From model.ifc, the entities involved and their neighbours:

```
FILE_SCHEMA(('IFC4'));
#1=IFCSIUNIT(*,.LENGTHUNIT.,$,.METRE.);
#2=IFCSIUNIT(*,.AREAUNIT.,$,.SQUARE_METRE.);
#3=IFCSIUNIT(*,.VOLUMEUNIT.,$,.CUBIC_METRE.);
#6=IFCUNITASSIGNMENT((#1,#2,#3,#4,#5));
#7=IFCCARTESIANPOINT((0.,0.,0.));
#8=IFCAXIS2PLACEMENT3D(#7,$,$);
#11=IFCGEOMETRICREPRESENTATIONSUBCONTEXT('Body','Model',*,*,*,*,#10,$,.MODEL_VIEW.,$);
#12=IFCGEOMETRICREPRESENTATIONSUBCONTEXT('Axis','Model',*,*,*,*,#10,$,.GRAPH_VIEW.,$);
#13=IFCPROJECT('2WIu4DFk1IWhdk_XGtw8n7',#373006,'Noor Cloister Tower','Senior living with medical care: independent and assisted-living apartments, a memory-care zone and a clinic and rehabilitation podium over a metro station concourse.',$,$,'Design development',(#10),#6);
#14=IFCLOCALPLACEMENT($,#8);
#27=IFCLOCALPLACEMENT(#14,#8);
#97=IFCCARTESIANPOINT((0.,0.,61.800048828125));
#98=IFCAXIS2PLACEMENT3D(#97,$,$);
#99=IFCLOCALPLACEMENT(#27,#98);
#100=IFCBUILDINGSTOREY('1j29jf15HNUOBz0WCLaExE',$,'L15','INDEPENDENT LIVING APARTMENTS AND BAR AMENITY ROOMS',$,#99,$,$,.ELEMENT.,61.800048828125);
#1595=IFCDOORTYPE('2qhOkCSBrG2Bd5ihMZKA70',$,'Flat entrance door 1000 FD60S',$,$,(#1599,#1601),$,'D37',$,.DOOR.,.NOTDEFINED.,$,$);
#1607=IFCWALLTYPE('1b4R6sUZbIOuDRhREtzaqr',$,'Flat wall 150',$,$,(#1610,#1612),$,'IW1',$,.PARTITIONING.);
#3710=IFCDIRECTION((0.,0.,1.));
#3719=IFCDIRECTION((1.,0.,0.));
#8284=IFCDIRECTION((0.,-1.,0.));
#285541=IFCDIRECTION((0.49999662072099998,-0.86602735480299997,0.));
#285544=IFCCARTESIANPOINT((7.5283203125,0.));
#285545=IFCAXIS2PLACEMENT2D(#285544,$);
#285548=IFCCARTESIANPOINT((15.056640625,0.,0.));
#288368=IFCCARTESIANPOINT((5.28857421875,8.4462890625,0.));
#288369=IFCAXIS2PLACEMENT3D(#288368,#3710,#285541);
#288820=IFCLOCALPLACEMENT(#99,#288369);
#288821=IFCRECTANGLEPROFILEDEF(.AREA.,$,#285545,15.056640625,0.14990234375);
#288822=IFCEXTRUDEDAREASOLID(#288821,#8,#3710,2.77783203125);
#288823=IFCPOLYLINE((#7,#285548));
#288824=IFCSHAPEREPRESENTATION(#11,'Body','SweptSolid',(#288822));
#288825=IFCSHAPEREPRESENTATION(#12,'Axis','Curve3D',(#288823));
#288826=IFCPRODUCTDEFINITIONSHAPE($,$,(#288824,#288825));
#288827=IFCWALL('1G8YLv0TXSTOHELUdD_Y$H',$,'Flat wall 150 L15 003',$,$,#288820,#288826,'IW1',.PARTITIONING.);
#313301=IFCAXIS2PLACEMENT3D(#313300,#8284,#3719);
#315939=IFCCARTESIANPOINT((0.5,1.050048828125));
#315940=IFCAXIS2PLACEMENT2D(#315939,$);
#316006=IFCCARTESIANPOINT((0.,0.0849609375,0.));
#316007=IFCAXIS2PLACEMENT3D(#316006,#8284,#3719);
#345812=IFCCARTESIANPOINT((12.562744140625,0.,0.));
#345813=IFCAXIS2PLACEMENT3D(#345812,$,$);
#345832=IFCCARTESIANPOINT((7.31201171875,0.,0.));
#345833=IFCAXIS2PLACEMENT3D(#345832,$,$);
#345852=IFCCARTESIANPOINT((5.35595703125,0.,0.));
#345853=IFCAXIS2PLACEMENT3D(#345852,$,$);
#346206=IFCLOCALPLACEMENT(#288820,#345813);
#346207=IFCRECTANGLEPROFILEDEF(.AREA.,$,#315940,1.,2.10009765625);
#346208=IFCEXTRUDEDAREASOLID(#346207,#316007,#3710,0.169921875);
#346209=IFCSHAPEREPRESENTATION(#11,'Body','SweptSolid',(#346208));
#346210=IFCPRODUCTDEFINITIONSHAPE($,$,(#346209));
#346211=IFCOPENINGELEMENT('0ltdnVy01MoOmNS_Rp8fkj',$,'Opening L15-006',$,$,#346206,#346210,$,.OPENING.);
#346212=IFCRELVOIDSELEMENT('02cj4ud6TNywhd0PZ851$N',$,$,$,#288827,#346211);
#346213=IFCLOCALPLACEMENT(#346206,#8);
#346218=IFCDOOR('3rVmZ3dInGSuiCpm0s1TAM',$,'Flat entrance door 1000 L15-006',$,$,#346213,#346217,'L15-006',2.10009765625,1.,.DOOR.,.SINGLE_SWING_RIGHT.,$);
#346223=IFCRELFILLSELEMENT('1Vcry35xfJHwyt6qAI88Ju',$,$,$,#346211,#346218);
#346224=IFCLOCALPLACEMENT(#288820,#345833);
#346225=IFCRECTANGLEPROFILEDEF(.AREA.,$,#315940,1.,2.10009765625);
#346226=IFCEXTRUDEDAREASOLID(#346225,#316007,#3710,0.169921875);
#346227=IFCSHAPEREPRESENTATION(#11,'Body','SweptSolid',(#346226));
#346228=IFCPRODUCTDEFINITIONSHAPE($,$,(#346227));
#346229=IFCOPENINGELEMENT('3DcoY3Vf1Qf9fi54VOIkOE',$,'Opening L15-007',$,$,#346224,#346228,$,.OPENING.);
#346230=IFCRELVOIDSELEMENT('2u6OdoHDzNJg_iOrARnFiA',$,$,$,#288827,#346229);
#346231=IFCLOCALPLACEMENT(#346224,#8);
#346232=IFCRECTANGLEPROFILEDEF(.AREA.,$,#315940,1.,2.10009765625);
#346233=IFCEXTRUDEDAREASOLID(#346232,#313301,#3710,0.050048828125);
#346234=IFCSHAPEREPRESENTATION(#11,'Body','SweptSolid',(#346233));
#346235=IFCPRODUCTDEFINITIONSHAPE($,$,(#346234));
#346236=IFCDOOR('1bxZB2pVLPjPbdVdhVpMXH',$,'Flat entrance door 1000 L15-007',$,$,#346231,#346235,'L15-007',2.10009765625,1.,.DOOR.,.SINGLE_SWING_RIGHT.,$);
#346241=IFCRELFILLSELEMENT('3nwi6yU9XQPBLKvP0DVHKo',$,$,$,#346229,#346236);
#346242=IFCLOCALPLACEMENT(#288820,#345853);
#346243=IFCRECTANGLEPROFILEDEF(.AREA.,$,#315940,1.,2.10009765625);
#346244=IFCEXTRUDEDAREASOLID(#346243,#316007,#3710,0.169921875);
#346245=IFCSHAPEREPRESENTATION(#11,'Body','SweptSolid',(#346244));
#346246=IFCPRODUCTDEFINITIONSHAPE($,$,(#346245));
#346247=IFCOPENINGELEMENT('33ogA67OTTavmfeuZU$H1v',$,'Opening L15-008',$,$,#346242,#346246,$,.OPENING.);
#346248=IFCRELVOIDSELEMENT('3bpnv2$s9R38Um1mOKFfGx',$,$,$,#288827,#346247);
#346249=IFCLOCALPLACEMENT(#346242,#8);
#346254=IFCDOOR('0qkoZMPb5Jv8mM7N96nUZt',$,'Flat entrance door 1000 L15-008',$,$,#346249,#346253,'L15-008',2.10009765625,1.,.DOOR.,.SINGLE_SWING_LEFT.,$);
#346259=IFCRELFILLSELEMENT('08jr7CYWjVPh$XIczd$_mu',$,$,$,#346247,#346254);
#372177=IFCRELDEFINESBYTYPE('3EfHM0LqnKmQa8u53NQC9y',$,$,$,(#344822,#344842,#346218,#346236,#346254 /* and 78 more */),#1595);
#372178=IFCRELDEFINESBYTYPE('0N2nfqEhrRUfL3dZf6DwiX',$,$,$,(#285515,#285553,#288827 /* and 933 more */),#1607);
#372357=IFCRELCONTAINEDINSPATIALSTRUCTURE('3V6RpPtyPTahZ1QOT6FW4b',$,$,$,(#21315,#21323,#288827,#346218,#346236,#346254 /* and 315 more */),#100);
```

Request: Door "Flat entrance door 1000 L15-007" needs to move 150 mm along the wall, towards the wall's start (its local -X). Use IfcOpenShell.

```python
import ifcopenshell
import ifcopenshell.api.geometry
import ifcopenshell.util.placement

model = ifcopenshell.open("model.ifc")

door = model.by_guid("1bxZB2pVLPjPbdVdhVpMXH")
opening = door.FillsVoids[0].RelatingOpeningElement
wall = opening.VoidsElements[0].RelatingBuildingElement

wall_matrix = ifcopenshell.util.placement.get_local_placement(wall.ObjectPlacement)
shift = wall_matrix[:3, 0] * -0.15
before = ifcopenshell.util.placement.get_local_placement(door.ObjectPlacement)[:3, 3].copy()

# The door is placed relative to its opening, so it follows when the opening moves.
matrix = ifcopenshell.util.placement.get_local_placement(opening.ObjectPlacement)
matrix[:3, 3] += shift
ifcopenshell.api.geometry.edit_object_placement(
    model, product=opening, matrix=matrix, is_si=False, should_transform_children=True
)

after = ifcopenshell.util.placement.get_local_placement(door.ObjectPlacement)[:3, 3]
print("door moved by", (after - before).round(3) + 0.0)

model.write("model_updated.ifc")
```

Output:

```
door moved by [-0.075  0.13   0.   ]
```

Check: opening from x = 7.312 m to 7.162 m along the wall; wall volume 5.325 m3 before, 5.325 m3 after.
